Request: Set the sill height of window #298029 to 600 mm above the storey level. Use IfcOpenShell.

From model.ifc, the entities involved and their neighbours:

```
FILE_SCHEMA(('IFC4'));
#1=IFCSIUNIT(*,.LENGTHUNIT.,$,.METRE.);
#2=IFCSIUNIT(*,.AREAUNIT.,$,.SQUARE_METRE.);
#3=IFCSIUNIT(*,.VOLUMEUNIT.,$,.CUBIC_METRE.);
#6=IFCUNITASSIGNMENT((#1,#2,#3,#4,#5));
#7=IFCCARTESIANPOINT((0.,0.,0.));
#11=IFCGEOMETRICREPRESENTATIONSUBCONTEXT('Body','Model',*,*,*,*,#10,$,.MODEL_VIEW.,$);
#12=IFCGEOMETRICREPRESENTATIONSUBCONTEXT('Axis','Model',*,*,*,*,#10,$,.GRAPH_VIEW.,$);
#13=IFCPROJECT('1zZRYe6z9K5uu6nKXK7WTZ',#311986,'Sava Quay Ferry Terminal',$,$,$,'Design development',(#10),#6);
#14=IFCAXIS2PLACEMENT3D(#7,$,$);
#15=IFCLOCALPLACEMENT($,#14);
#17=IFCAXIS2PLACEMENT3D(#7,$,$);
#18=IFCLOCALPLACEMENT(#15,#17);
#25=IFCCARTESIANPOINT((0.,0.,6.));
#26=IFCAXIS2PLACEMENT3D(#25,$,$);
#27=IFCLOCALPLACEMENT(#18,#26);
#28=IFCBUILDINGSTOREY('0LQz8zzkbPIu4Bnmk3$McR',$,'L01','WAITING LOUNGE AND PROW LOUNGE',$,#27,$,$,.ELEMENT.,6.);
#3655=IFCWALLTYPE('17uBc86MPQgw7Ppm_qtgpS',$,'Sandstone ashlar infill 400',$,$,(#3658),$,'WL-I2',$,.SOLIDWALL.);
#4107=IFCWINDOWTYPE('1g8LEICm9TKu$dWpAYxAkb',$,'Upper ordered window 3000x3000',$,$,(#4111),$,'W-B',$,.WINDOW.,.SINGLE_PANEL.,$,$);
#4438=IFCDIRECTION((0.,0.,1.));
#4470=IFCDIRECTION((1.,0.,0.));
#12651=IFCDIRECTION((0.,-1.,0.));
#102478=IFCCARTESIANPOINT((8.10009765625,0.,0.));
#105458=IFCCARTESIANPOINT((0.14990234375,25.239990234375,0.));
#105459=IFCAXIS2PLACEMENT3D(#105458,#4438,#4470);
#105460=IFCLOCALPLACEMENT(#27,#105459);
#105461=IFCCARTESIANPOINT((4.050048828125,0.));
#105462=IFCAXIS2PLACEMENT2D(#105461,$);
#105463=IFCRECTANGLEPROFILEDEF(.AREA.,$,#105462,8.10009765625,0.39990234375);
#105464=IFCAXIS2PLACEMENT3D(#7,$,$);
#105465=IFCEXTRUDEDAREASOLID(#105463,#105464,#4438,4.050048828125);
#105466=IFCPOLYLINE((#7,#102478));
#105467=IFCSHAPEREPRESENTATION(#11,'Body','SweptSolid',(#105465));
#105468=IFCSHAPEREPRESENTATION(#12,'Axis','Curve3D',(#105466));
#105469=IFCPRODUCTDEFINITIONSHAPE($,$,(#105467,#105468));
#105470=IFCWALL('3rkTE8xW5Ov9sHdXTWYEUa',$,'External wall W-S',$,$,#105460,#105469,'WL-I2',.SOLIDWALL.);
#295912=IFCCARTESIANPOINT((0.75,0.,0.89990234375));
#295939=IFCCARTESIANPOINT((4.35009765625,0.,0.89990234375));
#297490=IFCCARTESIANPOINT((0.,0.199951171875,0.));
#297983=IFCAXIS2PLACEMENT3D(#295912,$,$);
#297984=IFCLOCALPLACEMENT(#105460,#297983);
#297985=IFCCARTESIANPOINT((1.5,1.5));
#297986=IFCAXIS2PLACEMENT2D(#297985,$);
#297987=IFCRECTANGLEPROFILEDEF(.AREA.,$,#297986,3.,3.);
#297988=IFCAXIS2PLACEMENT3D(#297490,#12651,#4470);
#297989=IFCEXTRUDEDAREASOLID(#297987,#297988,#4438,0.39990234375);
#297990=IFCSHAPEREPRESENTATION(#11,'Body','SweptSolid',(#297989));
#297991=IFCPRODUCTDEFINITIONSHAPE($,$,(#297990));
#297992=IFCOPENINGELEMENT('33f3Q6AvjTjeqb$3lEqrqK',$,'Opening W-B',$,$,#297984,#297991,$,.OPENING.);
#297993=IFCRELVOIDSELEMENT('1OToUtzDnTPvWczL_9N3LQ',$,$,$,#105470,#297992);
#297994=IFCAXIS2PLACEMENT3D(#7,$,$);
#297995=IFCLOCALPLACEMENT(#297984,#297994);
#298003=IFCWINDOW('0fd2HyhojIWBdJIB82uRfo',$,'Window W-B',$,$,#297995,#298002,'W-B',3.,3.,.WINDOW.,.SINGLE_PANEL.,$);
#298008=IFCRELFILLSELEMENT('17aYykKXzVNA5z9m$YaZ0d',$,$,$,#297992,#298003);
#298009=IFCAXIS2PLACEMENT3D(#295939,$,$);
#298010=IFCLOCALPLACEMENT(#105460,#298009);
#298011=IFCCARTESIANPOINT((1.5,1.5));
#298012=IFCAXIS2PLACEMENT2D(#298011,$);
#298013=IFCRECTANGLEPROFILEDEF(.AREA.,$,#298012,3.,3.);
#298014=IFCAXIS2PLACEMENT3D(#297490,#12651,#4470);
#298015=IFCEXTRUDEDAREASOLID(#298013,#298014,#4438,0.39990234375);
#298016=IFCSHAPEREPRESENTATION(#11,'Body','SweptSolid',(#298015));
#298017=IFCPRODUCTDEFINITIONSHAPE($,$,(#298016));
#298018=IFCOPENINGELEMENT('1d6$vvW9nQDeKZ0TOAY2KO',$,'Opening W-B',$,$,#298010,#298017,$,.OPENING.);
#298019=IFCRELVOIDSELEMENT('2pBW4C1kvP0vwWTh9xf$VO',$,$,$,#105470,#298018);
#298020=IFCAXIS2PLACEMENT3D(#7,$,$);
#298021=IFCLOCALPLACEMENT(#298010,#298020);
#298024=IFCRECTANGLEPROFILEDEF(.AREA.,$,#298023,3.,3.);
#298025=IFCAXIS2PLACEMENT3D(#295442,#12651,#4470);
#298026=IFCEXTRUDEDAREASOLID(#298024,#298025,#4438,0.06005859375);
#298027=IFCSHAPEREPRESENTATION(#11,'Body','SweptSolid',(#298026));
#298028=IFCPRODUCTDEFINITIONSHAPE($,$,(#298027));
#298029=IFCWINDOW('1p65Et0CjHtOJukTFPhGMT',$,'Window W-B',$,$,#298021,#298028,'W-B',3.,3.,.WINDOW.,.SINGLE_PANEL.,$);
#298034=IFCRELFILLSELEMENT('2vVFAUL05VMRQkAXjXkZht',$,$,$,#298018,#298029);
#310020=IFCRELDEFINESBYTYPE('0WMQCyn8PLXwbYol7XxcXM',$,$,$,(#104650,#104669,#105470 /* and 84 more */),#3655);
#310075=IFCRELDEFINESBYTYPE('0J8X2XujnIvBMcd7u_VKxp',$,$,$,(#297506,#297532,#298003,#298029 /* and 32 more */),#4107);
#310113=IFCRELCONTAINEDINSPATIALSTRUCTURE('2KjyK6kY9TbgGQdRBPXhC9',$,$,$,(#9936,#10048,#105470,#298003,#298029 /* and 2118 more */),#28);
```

```python
import numpy as np
import ifcopenshell
import ifcopenshell.api.geometry
import ifcopenshell.geom
import ifcopenshell.util.element
import ifcopenshell.util.placement
import ifcopenshell.util.shape
import ifcopenshell.util.unit

model = ifcopenshell.open("model.ifc")
unit_scale = ifcopenshell.util.unit.calculate_unit_scale(model)

window = model.by_guid("1p65Et0CjHtOJukTFPhGMT")
opening = window.FillsVoids[0].RelatingOpeningElement
storey = ifcopenshell.util.element.get_container(window, ifc_class="IfcBuildingStorey")
level = ifcopenshell.util.placement.get_local_placement(storey.ObjectPlacement)[2, 3]

# The opening's origin need not be at the sill, so measure its lowest point.
shape = ifcopenshell.geom.create_shape(ifcopenshell.geom.settings(), opening)
bottom = ifcopenshell.util.shape.get_shape_bottom_elevation(shape, shape.geometry) / unit_scale
dz = level + 0.6 / unit_scale - bottom

shift = np.array([0.0, 0.0, dz])
# The window is placed relative to its opening, so it follows when the opening moves.
matrix = ifcopenshell.util.placement.get_local_placement(opening.ObjectPlacement)
matrix[:3, 3] += shift
ifcopenshell.api.geometry.edit_object_placement(
    model, product=opening, matrix=matrix, is_si=False, should_transform_children=True
)

print(f"moved by {dz * unit_scale:+.3f} m")

model.write("model-out.ifc")
```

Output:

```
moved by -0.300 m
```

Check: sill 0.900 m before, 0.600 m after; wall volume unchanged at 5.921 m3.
